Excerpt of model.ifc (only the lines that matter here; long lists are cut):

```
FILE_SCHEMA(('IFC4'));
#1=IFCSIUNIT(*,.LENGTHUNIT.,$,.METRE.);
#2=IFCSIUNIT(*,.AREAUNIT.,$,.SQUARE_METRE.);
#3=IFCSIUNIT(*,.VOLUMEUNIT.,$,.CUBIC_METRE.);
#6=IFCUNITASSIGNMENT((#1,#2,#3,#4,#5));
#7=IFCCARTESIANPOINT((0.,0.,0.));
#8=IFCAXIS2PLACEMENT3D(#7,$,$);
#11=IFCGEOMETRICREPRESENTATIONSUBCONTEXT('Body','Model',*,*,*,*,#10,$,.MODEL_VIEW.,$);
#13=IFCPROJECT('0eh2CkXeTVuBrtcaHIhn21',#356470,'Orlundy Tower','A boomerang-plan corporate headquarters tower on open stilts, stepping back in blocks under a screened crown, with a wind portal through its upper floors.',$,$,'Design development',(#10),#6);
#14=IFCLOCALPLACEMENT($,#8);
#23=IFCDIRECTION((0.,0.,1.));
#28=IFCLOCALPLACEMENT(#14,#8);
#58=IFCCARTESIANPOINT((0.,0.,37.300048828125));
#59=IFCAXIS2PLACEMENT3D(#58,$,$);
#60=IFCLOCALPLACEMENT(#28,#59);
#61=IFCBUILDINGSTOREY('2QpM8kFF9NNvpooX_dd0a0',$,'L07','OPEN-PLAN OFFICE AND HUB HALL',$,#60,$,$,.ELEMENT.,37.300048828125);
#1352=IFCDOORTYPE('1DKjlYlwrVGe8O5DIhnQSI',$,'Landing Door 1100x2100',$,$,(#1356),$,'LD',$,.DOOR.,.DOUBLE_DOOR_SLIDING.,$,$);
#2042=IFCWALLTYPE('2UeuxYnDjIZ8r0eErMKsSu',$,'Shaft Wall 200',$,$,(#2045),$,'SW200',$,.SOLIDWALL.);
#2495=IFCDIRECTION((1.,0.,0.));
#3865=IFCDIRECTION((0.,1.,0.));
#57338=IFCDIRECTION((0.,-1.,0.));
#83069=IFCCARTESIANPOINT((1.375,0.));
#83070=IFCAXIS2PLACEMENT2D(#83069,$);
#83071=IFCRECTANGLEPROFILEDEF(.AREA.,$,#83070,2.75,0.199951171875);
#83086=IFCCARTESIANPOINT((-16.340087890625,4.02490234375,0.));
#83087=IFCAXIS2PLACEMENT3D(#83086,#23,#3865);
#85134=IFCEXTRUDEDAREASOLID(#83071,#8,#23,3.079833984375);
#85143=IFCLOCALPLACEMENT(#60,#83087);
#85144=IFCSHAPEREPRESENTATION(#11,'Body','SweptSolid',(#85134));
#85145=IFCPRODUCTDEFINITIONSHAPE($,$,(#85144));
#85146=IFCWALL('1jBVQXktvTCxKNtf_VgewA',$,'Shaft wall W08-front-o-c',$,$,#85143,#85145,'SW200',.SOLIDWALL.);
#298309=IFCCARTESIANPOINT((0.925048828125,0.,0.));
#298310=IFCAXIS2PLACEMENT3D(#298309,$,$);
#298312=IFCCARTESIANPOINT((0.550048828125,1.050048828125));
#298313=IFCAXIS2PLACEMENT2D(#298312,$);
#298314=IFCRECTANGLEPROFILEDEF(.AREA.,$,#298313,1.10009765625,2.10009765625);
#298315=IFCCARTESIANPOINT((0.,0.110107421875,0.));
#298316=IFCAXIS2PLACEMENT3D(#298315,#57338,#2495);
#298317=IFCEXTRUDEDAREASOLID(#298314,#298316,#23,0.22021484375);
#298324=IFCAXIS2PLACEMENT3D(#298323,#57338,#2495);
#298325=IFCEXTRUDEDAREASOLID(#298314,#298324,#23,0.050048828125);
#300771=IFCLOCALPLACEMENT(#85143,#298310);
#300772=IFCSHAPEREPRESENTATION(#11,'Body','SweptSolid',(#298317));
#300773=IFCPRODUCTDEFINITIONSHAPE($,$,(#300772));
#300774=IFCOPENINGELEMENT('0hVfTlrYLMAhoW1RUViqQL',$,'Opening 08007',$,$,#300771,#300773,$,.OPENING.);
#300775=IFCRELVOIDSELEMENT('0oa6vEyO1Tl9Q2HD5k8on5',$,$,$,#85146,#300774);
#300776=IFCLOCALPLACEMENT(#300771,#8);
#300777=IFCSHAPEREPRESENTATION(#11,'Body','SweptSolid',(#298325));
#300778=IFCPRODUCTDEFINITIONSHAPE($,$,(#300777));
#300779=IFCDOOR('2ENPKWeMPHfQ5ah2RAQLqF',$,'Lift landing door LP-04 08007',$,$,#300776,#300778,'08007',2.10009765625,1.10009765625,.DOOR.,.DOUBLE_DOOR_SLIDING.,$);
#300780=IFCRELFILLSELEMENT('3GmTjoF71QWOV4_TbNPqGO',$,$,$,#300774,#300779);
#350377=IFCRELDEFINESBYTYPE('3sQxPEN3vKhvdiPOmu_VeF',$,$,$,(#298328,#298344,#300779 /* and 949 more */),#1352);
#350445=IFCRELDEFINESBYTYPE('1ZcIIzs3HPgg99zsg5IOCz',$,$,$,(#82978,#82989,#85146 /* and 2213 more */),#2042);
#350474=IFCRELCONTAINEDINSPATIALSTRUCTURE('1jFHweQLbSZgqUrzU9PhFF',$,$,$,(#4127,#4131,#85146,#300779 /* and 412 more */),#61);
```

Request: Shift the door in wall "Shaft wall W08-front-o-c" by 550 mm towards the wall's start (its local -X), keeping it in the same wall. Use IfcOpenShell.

```python
import ifcopenshell
import ifcopenshell.api.geometry
import ifcopenshell.util.placement
import ifcopenshell.util.unit

model = ifcopenshell.open("model.ifc")
unit_scale = ifcopenshell.util.unit.calculate_unit_scale(model)

door = model.by_guid("2ENPKWeMPHfQ5ah2RAQLqF")
opening = door.FillsVoids[0].RelatingOpeningElement
wall = opening.VoidsElements[0].RelatingBuildingElement

wall_matrix = ifcopenshell.util.placement.get_local_placement(wall.ObjectPlacement)
shift = wall_matrix[:3, 0] * -0.55 / unit_scale
before = ifcopenshell.util.placement.get_local_placement(door.ObjectPlacement)[:3, 3].copy()

# The door is placed relative to its opening, so it follows when the opening moves.
matrix = ifcopenshell.util.placement.get_local_placement(opening.ObjectPlacement)
matrix[:3, 3] += shift
ifcopenshell.api.geometry.edit_object_placement(
    model, product=opening, matrix=matrix, is_si=False, should_transform_children=True
)

after = ifcopenshell.util.placement.get_local_placement(door.ObjectPlacement)[:3, 3]
print("door moved by", (after - before).round(3) + 0.0)

model.write("model_edited.ifc")
```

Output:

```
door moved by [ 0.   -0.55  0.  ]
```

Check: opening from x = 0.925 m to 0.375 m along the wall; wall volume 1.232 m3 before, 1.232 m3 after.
